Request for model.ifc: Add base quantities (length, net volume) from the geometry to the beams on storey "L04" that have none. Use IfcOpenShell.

First a look at what the model holds.

```python
import ifcopenshell
import ifcopenshell.util.element
import ifcopenshell.util.unit

model = ifcopenshell.open("model.ifc")
print(model.schema)
for unit_type in ("LENGTHUNIT", "AREAUNIT", "VOLUMEUNIT"):
    print(unit_type, ifcopenshell.util.unit.calculate_unit_scale(model, unit_type))
storey = next(s for s in model.by_type("IfcBuildingStorey") if s.Name == "L04")
beams = [e for e in ifcopenshell.util.element.get_decomposition(storey) if e.is_a("IfcBeam")]
for e in sorted(beams, key=lambda e: e.id()):
    print(e.id(), e.is_a(), e.Name, list(ifcopenshell.util.element.get_psets(e, qtos_only=True)), sep=" | ")
```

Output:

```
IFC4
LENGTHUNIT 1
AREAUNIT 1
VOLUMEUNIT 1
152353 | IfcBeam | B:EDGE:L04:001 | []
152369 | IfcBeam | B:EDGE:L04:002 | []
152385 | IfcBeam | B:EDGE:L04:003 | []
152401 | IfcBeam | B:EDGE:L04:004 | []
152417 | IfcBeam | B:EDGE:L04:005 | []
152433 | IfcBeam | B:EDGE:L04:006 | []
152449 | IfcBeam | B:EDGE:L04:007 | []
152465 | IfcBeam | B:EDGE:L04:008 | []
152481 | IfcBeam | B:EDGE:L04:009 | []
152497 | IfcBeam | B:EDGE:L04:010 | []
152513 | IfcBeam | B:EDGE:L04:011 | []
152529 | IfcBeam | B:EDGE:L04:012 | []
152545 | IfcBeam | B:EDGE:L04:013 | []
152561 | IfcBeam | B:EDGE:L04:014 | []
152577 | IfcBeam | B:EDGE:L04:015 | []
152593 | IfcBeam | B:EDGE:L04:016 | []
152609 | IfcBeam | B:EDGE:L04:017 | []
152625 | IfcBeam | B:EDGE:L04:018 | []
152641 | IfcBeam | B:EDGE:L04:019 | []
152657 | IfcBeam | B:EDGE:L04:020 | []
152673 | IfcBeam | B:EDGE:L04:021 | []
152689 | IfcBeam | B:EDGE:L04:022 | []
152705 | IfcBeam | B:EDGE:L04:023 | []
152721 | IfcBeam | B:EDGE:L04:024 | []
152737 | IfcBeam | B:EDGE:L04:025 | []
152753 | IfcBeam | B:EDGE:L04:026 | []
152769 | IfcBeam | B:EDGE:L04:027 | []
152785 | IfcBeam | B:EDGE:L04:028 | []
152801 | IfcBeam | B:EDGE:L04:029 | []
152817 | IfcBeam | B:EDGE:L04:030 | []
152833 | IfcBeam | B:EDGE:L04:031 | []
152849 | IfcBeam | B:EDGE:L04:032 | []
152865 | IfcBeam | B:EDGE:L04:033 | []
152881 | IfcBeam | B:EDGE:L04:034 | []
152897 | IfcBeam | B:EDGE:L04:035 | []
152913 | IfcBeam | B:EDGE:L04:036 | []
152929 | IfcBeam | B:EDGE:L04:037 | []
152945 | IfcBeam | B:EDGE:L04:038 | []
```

```python
import ifcopenshell
import ifcopenshell.api.pset
import ifcopenshell.geom
import ifcopenshell.util.element
import ifcopenshell.util.shape
import ifcopenshell.util.unit

model = ifcopenshell.open("model.ifc")
unit_scale = ifcopenshell.util.unit.calculate_unit_scale(model)
volume_scale = ifcopenshell.util.unit.calculate_unit_scale(model, "VOLUMEUNIT")
settings = ifcopenshell.geom.settings()

storey = next(s for s in model.by_type("IfcBuildingStorey") if s.Name == "L04")
beams = [e for e in ifcopenshell.util.element.get_decomposition(storey) if e.is_a("IfcBeam")]

for e in sorted(beams, key=lambda e: e.id()):
    if ifcopenshell.util.element.get_psets(e, qtos_only=True, should_inherit=False):
        continue
    # Geometry comes back in metres, in the element's own axes.
    shape = ifcopenshell.geom.create_shape(settings, e)
    values = {
        "Length": ifcopenshell.util.shape.get_max_xyz(shape.geometry) / unit_scale,
        "NetVolume": ifcopenshell.util.shape.get_volume(shape.geometry) / volume_scale,
    }
    qto = ifcopenshell.api.pset.add_qto(model, product=e, name="Qto_BeamBaseQuantities")
    ifcopenshell.api.pset.edit_qto(model, qto=qto, properties=values)
    print(e.id(), {k: round(v, 3) for k, v in values.items()})

model.write("model_rev.ifc")
```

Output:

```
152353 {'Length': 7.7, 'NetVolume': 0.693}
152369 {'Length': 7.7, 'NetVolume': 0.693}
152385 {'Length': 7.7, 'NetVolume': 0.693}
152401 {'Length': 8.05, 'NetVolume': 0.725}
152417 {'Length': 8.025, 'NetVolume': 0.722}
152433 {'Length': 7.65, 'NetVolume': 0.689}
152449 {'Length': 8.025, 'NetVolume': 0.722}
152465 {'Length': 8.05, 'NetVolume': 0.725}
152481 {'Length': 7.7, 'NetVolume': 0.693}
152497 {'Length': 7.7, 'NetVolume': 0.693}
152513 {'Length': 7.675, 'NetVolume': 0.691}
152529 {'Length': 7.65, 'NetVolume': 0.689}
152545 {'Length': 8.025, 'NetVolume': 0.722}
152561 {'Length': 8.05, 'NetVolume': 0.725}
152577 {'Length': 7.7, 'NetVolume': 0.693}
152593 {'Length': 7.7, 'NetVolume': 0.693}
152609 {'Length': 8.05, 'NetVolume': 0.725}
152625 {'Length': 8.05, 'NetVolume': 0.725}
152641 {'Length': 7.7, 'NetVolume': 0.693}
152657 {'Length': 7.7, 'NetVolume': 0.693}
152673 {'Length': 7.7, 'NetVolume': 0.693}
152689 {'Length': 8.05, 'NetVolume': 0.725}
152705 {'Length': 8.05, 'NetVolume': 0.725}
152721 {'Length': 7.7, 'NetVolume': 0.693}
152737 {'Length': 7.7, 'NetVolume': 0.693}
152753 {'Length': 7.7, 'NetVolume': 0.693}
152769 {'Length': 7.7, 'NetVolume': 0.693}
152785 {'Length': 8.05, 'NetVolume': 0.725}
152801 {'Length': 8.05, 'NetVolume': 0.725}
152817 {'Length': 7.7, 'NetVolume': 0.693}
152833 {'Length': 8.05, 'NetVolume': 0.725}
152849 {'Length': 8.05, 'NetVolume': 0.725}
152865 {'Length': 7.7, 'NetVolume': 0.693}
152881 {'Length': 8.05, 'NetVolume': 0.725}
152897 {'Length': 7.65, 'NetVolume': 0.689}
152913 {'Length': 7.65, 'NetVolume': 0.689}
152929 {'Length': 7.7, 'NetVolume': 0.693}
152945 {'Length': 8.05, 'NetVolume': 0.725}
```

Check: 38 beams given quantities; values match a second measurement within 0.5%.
